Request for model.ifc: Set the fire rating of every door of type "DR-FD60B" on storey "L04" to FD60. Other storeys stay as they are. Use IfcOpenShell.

First a look at what the model holds.

```python
import ifcopenshell
import ifcopenshell.util.element

model = ifcopenshell.open("model.ifc")
print(model.schema)
storey = next(s for s in model.by_type("IfcBuildingStorey") if s.Name == "L04")
doors = [e for e in ifcopenshell.util.element.get_decomposition(storey) if e.is_a("IfcDoor")]
seen = {}
for e in doors:
    element_type = ifcopenshell.util.element.get_type(e)
    key = (element_type.Name if element_type != e and element_type else None, ifcopenshell.util.element.get_pset(e, "Pset_DoorCommon", "FireRating"))
    seen[key] = seen.get(key, 0) + 1
for (name, value), count in sorted(seen.items(), key=str):
    print(count, "x", name, "|", value)
```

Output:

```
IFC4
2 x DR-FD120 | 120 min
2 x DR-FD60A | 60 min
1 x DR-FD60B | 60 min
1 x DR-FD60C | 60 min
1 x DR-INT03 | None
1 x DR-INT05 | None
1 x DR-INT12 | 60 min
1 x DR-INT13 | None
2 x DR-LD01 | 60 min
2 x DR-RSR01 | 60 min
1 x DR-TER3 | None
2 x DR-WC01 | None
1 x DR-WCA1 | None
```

```python
import ifcopenshell
import ifcopenshell.api.pset
import ifcopenshell.util.element

model = ifcopenshell.open("model.ifc")

storey = next(s for s in model.by_type("IfcBuildingStorey") if s.Name == "L04")
doors = [e for e in ifcopenshell.util.element.get_decomposition(storey) if e.is_a("IfcDoor")]

count = 0
for e in doors:
    element_type = ifcopenshell.util.element.get_type(e)
    if element_type in (None, e) or element_type.Name != "DR-FD60B":
        continue
    # add_pset returns the element's existing set when there is one.
    pset = ifcopenshell.api.pset.add_pset(model, product=e, name="Pset_DoorCommon")
    ifcopenshell.api.pset.edit_pset(model, pset=pset, properties={"FireRating": "FD60"})
    count += 1

print(count, "doors updated")

model.write("model-out.ifc")
```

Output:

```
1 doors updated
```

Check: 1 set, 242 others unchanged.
